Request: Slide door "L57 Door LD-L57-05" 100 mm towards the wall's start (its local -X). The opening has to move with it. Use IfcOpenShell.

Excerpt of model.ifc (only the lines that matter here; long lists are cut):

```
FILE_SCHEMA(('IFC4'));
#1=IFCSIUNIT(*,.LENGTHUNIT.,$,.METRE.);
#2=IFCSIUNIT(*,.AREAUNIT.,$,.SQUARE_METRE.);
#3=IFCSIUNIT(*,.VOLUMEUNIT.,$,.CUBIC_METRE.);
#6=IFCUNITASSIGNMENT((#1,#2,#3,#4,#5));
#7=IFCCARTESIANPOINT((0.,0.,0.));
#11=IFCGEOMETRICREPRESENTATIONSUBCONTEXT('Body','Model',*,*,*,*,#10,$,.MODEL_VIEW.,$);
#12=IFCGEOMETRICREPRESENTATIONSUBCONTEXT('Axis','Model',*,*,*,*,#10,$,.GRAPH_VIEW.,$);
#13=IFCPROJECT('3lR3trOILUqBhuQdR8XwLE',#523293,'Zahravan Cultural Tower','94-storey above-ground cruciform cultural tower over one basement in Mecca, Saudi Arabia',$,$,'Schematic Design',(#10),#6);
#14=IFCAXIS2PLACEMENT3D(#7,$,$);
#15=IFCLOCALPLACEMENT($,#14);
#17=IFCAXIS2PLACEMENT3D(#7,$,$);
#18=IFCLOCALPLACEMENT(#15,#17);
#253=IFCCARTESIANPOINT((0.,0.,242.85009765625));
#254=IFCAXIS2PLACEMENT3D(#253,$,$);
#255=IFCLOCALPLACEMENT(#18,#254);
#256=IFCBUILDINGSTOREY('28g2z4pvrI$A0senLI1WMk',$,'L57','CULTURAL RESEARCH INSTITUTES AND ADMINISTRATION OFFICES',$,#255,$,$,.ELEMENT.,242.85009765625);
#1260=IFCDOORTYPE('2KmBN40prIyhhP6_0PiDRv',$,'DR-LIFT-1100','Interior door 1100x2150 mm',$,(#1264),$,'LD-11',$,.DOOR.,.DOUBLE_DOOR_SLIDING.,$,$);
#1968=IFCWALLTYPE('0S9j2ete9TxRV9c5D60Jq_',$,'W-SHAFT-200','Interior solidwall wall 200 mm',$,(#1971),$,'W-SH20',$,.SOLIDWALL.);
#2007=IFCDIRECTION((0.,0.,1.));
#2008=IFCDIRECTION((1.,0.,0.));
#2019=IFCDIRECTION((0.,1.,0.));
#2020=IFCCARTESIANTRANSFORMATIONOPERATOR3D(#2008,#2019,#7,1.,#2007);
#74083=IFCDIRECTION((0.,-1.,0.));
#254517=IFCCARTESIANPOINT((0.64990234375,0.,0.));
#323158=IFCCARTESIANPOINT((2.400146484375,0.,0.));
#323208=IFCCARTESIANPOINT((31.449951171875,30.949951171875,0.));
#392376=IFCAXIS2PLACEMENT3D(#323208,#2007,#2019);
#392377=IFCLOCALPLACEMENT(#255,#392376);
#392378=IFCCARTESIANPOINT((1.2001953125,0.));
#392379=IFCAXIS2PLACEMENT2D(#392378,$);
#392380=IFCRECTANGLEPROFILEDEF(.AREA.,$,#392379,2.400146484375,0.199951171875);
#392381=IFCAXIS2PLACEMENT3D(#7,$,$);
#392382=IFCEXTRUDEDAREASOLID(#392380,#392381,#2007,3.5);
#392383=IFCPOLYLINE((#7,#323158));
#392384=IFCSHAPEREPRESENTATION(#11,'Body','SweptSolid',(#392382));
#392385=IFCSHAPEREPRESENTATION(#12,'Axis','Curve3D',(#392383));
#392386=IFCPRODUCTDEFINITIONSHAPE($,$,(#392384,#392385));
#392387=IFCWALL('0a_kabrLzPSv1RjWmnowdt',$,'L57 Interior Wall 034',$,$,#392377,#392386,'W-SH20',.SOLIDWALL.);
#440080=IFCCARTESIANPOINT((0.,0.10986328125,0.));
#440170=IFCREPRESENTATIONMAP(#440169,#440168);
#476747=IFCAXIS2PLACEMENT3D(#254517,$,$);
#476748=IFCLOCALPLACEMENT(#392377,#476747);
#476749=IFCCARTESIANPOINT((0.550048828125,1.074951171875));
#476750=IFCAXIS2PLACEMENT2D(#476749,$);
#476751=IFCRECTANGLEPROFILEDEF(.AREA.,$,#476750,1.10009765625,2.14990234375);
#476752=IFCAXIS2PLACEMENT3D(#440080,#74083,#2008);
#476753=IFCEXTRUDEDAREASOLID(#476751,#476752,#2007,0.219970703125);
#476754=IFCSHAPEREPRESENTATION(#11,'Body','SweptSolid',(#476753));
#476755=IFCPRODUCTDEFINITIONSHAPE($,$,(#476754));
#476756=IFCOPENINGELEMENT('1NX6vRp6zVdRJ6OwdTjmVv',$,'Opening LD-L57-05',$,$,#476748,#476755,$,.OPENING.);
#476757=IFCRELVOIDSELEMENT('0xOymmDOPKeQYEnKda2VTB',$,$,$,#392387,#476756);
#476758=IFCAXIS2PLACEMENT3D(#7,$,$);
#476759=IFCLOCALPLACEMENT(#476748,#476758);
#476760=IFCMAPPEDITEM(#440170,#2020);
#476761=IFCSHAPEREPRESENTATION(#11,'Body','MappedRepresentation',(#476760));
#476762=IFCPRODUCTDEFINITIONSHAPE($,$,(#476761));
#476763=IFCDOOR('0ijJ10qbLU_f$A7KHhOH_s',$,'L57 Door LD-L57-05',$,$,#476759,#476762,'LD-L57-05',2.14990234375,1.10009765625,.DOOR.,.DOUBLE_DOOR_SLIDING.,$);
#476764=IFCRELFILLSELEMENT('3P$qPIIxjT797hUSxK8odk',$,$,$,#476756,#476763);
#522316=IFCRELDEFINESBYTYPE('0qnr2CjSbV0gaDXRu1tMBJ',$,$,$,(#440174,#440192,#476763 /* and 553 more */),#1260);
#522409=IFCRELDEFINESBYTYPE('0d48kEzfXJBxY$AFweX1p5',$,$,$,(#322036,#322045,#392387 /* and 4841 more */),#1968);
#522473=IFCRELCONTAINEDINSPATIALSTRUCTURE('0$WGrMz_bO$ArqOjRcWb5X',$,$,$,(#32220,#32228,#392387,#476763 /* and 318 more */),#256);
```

```python
import ifcopenshell
import ifcopenshell.api.geometry
import ifcopenshell.util.placement

model = ifcopenshell.open("model.ifc")

door = model.by_guid("0ijJ10qbLU_f$A7KHhOH_s")
opening = door.FillsVoids[0].RelatingOpeningElement
wall = opening.VoidsElements[0].RelatingBuildingElement

wall_matrix = ifcopenshell.util.placement.get_local_placement(wall.ObjectPlacement)
shift = wall_matrix[:3, 0] * -0.1
before = ifcopenshell.util.placement.get_local_placement(door.ObjectPlacement)[:3, 3].copy()

# The door is placed relative to its opening, so it follows when the opening moves.
matrix = ifcopenshell.util.placement.get_local_placement(opening.ObjectPlacement)
matrix[:3, 3] += shift
ifcopenshell.api.geometry.edit_object_placement(
    model, product=opening, matrix=matrix, is_si=False, should_transform_children=True
)

after = ifcopenshell.util.placement.get_local_placement(door.ObjectPlacement)[:3, 3]
print("door moved by", (after - before).round(3) + 0.0)

model.write("model_edited.ifc")
```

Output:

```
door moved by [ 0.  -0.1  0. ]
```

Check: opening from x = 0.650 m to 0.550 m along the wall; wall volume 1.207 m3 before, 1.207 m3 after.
